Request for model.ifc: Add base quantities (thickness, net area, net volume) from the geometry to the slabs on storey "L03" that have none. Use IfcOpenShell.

First a look at what the model holds.

```python
import ifcopenshell
import ifcopenshell.util.element
import ifcopenshell.util.unit

model = ifcopenshell.open("model.ifc")
print(model.schema)
for unit_type in ("LENGTHUNIT", "AREAUNIT", "VOLUMEUNIT"):
    print(unit_type, ifcopenshell.util.unit.calculate_unit_scale(model, unit_type))
storey = next(s for s in model.by_type("IfcBuildingStorey") if s.Name == "L03")
slabs = [e for e in ifcopenshell.util.element.get_decomposition(storey) if e.is_a("IfcSlab")]
for e in sorted(slabs, key=lambda e: e.id()):
    print(e.id(), e.is_a(), e.Name, list(ifcopenshell.util.element.get_psets(e, qtos_only=True)), sep=" | ")
```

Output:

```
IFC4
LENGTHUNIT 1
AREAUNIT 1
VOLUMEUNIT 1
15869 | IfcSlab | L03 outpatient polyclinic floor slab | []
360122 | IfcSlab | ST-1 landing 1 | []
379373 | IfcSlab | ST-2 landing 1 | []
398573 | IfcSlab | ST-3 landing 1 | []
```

```python
import ifcopenshell
import ifcopenshell.api.pset
import ifcopenshell.geom
import ifcopenshell.util.element
import ifcopenshell.util.shape
import ifcopenshell.util.unit

model = ifcopenshell.open("model.ifc")
unit_scale = ifcopenshell.util.unit.calculate_unit_scale(model)
area_scale = ifcopenshell.util.unit.calculate_unit_scale(model, "AREAUNIT")
volume_scale = ifcopenshell.util.unit.calculate_unit_scale(model, "VOLUMEUNIT")
settings = ifcopenshell.geom.settings()

storey = next(s for s in model.by_type("IfcBuildingStorey") if s.Name == "L03")
slabs = [e for e in ifcopenshell.util.element.get_decomposition(storey) if e.is_a("IfcSlab")]

for e in sorted(slabs, key=lambda e: e.id()):
    if ifcopenshell.util.element.get_psets(e, qtos_only=True, should_inherit=False):
        continue
    # Geometry comes back in metres, in the element's own axes.
    shape = ifcopenshell.geom.create_shape(settings, e)
    values = {
        "Width": ifcopenshell.util.shape.get_z(shape.geometry) / unit_scale,
        "NetArea": ifcopenshell.util.shape.get_footprint_area(shape.geometry) / area_scale,
        "NetVolume": ifcopenshell.util.shape.get_volume(shape.geometry) / volume_scale,
    }
    qto = ifcopenshell.api.pset.add_qto(model, product=e, name="Qto_SlabBaseQuantities")
    ifcopenshell.api.pset.edit_qto(model, qto=qto, properties=values)
    print(e.id(), {k: round(v, 3) for k, v in values.items()})

model.write("model_updated.ifc")
```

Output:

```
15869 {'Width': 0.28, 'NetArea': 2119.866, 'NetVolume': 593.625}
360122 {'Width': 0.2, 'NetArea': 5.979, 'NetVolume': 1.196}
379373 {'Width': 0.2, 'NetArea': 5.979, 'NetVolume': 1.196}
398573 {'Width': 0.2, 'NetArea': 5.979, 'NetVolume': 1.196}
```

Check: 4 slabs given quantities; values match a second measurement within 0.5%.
